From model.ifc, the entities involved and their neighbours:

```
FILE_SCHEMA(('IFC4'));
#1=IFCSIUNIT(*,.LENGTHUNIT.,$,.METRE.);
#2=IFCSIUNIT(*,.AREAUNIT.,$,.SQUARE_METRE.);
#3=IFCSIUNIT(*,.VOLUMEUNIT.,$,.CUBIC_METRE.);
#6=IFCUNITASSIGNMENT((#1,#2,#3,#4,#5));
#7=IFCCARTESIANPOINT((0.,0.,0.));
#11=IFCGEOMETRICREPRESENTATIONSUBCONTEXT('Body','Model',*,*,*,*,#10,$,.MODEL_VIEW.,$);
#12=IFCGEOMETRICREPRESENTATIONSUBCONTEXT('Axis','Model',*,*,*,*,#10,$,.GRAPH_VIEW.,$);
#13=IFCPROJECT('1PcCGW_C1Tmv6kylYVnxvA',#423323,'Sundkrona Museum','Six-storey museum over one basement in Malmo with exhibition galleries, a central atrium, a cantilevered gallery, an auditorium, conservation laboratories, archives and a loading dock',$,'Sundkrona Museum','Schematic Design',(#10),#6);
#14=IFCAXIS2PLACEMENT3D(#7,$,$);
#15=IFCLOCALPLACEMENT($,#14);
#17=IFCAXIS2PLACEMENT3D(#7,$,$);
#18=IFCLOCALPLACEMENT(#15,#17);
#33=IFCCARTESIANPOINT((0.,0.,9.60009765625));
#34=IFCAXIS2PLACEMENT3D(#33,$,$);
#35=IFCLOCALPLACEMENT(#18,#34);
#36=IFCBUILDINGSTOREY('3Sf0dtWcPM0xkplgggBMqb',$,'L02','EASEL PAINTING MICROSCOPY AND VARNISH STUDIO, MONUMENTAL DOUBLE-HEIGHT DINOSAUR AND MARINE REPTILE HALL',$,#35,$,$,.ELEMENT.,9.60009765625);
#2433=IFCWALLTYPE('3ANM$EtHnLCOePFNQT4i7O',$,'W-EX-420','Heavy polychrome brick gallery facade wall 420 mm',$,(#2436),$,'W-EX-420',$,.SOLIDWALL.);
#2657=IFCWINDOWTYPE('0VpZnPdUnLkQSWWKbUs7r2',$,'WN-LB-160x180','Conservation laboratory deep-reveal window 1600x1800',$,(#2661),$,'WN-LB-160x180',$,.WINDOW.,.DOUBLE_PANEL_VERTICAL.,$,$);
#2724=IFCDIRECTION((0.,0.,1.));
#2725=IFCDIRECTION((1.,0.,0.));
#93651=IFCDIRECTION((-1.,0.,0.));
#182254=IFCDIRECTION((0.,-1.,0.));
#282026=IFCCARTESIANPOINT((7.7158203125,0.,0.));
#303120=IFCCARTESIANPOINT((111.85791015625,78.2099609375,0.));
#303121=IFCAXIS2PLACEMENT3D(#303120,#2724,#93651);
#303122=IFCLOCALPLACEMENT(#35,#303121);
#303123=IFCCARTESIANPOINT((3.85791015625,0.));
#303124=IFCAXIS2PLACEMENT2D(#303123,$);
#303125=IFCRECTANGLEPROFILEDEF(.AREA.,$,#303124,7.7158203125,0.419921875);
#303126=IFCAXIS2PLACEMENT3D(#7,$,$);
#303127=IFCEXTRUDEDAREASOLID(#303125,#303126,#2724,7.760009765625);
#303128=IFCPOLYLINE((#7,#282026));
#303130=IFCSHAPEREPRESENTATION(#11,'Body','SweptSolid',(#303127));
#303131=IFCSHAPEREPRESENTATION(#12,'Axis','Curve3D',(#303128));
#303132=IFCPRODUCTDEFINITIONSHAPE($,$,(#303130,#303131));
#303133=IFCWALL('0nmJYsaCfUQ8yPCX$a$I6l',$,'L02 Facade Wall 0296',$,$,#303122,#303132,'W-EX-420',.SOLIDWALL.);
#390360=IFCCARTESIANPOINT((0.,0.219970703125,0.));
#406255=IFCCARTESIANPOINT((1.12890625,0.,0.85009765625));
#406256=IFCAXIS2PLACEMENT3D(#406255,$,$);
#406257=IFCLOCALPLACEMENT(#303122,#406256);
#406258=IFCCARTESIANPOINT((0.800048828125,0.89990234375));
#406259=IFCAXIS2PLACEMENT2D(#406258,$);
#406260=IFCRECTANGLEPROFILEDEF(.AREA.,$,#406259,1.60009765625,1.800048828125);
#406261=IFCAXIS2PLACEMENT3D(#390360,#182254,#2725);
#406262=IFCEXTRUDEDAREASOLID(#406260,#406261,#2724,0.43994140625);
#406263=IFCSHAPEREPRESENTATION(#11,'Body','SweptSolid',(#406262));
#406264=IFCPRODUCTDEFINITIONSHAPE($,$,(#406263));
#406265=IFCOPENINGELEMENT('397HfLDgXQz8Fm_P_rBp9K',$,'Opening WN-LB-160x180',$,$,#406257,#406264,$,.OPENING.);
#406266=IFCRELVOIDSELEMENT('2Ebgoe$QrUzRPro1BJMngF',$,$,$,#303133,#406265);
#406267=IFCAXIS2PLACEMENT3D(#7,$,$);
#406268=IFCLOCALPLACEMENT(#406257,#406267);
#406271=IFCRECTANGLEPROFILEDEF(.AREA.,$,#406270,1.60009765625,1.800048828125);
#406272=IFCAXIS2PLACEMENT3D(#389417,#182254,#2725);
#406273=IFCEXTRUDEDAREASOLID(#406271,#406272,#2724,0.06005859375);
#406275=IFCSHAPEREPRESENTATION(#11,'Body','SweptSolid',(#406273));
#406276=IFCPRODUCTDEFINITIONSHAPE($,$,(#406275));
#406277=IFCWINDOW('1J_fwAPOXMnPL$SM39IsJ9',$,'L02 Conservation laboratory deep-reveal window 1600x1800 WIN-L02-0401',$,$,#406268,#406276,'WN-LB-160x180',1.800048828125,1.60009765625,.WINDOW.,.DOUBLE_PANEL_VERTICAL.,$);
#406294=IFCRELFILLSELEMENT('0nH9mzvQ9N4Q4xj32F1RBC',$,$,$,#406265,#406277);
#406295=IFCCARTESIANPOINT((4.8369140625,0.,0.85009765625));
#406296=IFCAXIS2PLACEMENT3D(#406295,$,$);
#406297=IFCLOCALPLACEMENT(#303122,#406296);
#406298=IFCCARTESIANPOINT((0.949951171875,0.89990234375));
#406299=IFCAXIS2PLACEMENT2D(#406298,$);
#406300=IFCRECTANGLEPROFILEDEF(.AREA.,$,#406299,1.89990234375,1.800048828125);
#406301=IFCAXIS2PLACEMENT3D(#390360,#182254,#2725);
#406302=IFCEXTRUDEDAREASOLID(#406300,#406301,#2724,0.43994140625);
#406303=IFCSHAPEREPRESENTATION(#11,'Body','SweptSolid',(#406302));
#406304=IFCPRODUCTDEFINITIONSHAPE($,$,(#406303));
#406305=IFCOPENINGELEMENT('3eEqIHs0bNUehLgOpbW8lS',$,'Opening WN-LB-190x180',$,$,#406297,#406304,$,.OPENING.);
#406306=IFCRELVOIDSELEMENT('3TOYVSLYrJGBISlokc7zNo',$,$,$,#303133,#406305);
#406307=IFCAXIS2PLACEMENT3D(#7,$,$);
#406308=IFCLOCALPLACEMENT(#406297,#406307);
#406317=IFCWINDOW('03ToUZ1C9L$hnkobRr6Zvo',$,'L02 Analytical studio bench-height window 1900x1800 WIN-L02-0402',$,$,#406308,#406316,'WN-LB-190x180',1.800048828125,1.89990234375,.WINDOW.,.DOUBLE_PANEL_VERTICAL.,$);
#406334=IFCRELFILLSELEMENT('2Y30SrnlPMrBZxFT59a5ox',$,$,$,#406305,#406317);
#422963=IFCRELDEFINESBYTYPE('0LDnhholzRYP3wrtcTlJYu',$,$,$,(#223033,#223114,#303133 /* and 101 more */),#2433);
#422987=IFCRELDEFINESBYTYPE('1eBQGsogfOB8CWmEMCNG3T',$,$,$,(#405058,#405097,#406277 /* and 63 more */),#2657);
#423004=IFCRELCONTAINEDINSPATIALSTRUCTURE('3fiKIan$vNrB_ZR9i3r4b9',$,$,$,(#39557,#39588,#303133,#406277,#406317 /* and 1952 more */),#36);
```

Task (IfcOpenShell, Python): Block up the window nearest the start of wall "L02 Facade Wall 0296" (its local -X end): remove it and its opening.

```python
import ifcopenshell
import ifcopenshell.api.feature
import ifcopenshell.api.root
import ifcopenshell.geom
import ifcopenshell.util.shape

model = ifcopenshell.open("model.ifc")
settings = ifcopenshell.geom.settings()


def volume(element):
    """Net volume in cubic metres, openings subtracted."""
    shape = ifcopenshell.geom.create_shape(settings, element)
    return ifcopenshell.util.shape.get_volume(shape.geometry)


window = model.by_id(406277)
opening = window.FillsVoids[0].RelatingOpeningElement
wall = opening.VoidsElements[0].RelatingBuildingElement
before = volume(wall)

ifcopenshell.api.root.remove_product(model, product=window)
ifcopenshell.api.feature.remove_feature(model, feature=opening)

after = volume(wall)

print(f"wall volume {before:.3f} -> {after:.3f} m3")

model.write("model_rev.ifc")
```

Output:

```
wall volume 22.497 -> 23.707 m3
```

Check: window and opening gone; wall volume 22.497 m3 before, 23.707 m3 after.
